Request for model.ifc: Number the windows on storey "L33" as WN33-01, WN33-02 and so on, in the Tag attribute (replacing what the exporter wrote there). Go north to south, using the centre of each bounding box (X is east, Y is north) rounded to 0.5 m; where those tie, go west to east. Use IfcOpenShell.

First a look at what the model holds.

```python
import ifcopenshell
import ifcopenshell.util.element
import ifcopenshell.util.placement

model = ifcopenshell.open("model.ifc")
print(model.schema)
storey = next(s for s in model.by_type("IfcBuildingStorey") if s.Name == "L33")
windows = [e for e in ifcopenshell.util.element.get_decomposition(storey) if e.is_a("IfcWindow")]
for e in sorted(windows, key=lambda e: e.id()):
    origin = ifcopenshell.util.placement.get_local_placement(e.ObjectPlacement)[:3, 3]
    print(e.id(), e.Tag, e.Name, origin.round(2) + 0.0, sep=" | ")
```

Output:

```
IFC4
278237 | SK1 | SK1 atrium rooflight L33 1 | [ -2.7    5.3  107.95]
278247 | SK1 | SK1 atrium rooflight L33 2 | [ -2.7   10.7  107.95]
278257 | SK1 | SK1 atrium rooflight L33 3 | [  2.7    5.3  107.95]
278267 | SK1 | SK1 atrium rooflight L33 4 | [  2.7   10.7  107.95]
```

```python
import ifcopenshell
import ifcopenshell.geom
import ifcopenshell.util.element
import ifcopenshell.util.shape

model = ifcopenshell.open("model.ifc")
settings = ifcopenshell.geom.settings()
settings.set("use-world-coords", True)


def centre(element):
    shape = ifcopenshell.geom.create_shape(settings, element)
    return ifcopenshell.util.shape.get_bbox_centroid(shape.geometry)


storey = next(s for s in model.by_type("IfcBuildingStorey") if s.Name == "L33")
windows = [e for e in ifcopenshell.util.element.get_decomposition(storey) if e.is_a("IfcWindow")]

# Insertion points can sit at a corner or the storey origin, so sort by the geometry (in metres).
centres = {e: centre(e) for e in windows}
windows.sort(key=lambda e: (-round(centres[e][1] / 0.5), centres[e][0]))

for i, e in enumerate(windows, start=1):
    number = f"WN33-{i:02d}"
    e.Tag = number
    print(e.id(), number)

model.write("model_updated.ifc")
```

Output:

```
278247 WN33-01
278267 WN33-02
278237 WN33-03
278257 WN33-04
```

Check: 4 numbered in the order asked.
